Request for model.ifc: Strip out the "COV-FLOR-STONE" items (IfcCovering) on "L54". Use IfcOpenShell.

First a look at what the model holds.

```python
import ifcopenshell
import ifcopenshell.util.element

model = ifcopenshell.open("model.ifc")
print(model.schema)
storey = next(s for s in model.by_type("IfcBuildingStorey") if s.Name == "L54")
coverings = [e for e in ifcopenshell.util.element.get_decomposition(storey) if e.is_a("IfcCovering")]
seen = {}
for e in coverings:
    element_type = ifcopenshell.util.element.get_type(e)
    name = element_type.Name if element_type not in (None, e) else None
    seen[name] = seen.get(name, 0) + 1
for name, count in sorted(seen.items(), key=str):
    print(count, "x", name)
```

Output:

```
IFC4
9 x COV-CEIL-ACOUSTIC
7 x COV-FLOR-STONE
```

```python
import ifcopenshell
import ifcopenshell.api.root
import ifcopenshell.util.element

model = ifcopenshell.open("model.ifc")

storey = next(s for s in model.by_type("IfcBuildingStorey") if s.Name == "L54")
coverings = [e for e in ifcopenshell.util.element.get_decomposition(storey) if e.is_a("IfcCovering")]
targets = [e for e in coverings if (t := ifcopenshell.util.element.get_type(e)) not in (None, e) and t.Name == "COV-FLOR-STONE"]

for e in targets:
    ifcopenshell.api.root.remove_product(model, product=e)
print(len(targets), "removed")

model.write("model_rev.ifc")
```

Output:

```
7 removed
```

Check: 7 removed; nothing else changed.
